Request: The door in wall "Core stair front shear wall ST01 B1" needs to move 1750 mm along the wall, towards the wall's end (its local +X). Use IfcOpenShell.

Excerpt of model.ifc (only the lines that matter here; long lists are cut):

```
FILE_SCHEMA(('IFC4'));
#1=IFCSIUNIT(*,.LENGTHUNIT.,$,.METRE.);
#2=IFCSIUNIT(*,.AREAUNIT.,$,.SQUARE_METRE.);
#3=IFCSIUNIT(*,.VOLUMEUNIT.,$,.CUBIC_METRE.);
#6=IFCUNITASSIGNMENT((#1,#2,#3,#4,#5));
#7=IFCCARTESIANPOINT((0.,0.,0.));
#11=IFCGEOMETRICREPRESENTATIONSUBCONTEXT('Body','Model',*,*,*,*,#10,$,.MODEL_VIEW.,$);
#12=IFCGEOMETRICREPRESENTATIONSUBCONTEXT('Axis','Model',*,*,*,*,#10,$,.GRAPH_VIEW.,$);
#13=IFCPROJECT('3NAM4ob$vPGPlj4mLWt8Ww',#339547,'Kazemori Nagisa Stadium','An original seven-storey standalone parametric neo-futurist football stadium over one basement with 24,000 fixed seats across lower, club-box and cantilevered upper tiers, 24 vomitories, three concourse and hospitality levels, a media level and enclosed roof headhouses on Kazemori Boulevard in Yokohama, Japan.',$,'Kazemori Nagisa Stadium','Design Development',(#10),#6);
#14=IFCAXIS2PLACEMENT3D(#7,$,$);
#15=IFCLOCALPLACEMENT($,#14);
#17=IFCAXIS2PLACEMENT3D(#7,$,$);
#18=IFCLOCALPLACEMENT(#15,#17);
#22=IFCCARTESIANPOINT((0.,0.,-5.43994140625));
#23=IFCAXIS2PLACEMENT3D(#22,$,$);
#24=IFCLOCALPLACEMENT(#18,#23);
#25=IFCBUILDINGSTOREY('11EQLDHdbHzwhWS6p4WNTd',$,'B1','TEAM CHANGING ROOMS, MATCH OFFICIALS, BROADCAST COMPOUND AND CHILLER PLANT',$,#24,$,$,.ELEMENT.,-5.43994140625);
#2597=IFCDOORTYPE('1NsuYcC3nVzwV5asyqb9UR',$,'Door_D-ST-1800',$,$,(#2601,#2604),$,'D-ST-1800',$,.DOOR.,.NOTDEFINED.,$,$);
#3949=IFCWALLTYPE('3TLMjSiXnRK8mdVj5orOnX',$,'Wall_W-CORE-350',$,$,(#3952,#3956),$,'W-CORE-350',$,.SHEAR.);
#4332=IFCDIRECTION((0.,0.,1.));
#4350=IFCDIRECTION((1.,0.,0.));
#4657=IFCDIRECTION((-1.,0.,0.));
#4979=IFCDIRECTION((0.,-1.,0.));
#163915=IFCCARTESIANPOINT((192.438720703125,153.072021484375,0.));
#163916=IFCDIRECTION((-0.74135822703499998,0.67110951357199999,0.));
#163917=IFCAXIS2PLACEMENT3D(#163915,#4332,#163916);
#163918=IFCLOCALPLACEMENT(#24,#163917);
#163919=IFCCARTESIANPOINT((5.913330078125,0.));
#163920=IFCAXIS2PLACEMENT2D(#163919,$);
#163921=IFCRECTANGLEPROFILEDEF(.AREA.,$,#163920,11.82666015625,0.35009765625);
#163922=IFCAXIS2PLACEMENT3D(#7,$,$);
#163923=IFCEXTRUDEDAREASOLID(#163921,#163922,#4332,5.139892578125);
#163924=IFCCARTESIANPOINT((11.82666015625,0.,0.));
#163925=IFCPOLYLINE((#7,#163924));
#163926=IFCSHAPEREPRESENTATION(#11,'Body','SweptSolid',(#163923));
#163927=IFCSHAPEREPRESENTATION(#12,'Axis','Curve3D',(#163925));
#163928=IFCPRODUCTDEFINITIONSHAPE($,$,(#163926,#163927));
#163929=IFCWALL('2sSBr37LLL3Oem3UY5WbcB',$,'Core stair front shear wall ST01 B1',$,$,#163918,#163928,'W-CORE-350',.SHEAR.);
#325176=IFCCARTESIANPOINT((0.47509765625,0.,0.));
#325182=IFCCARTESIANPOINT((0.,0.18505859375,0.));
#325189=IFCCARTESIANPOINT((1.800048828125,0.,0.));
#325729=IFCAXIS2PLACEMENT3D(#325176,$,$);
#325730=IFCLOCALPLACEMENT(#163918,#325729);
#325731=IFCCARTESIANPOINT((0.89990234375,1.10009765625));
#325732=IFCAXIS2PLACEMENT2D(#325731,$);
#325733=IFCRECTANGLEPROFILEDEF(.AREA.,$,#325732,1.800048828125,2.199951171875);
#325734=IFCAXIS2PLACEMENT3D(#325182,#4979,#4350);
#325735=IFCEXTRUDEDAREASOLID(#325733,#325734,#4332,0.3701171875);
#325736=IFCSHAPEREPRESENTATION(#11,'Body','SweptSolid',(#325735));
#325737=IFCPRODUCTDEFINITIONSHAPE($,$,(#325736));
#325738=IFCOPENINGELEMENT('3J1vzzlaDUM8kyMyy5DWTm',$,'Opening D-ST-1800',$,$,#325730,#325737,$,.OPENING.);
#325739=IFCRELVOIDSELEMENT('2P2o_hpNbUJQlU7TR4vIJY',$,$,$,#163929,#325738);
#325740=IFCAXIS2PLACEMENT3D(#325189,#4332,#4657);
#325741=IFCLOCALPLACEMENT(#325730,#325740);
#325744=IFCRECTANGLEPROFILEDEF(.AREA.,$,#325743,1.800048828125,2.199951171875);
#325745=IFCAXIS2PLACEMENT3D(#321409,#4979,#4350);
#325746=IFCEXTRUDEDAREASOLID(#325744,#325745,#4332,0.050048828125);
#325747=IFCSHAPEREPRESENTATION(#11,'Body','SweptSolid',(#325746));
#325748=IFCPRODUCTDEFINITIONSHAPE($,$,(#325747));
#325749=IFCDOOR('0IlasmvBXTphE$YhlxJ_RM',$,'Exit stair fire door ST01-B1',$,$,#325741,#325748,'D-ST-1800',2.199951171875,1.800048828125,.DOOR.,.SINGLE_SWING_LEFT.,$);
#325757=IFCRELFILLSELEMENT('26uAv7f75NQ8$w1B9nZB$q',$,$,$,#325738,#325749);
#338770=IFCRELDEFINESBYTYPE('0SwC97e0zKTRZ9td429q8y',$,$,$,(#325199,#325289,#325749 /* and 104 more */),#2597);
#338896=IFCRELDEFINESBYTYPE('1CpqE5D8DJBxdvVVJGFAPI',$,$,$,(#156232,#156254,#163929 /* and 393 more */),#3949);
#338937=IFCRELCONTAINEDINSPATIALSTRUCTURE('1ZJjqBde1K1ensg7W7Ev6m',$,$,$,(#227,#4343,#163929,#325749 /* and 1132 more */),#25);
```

```python
import ifcopenshell
import ifcopenshell.api.geometry
import ifcopenshell.util.placement

model = ifcopenshell.open("model.ifc")

door = model.by_id(325749)
opening = door.FillsVoids[0].RelatingOpeningElement
wall = opening.VoidsElements[0].RelatingBuildingElement

wall_matrix = ifcopenshell.util.placement.get_local_placement(wall.ObjectPlacement)
shift = wall_matrix[:3, 0] * 1.75
before = ifcopenshell.util.placement.get_local_placement(door.ObjectPlacement)[:3, 3].copy()

# The door is placed relative to its opening, so it follows when the opening moves.
matrix = ifcopenshell.util.placement.get_local_placement(opening.ObjectPlacement)
matrix[:3, 3] += shift
ifcopenshell.api.geometry.edit_object_placement(
    model, product=opening, matrix=matrix, is_si=False, should_transform_children=True
)

after = ifcopenshell.util.placement.get_local_placement(door.ObjectPlacement)[:3, 3]
print("door moved by", (after - before).round(3) + 0.0)

model.write("model-out.ifc")
```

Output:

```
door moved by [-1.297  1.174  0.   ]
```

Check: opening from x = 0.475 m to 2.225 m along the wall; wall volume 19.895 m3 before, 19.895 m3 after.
